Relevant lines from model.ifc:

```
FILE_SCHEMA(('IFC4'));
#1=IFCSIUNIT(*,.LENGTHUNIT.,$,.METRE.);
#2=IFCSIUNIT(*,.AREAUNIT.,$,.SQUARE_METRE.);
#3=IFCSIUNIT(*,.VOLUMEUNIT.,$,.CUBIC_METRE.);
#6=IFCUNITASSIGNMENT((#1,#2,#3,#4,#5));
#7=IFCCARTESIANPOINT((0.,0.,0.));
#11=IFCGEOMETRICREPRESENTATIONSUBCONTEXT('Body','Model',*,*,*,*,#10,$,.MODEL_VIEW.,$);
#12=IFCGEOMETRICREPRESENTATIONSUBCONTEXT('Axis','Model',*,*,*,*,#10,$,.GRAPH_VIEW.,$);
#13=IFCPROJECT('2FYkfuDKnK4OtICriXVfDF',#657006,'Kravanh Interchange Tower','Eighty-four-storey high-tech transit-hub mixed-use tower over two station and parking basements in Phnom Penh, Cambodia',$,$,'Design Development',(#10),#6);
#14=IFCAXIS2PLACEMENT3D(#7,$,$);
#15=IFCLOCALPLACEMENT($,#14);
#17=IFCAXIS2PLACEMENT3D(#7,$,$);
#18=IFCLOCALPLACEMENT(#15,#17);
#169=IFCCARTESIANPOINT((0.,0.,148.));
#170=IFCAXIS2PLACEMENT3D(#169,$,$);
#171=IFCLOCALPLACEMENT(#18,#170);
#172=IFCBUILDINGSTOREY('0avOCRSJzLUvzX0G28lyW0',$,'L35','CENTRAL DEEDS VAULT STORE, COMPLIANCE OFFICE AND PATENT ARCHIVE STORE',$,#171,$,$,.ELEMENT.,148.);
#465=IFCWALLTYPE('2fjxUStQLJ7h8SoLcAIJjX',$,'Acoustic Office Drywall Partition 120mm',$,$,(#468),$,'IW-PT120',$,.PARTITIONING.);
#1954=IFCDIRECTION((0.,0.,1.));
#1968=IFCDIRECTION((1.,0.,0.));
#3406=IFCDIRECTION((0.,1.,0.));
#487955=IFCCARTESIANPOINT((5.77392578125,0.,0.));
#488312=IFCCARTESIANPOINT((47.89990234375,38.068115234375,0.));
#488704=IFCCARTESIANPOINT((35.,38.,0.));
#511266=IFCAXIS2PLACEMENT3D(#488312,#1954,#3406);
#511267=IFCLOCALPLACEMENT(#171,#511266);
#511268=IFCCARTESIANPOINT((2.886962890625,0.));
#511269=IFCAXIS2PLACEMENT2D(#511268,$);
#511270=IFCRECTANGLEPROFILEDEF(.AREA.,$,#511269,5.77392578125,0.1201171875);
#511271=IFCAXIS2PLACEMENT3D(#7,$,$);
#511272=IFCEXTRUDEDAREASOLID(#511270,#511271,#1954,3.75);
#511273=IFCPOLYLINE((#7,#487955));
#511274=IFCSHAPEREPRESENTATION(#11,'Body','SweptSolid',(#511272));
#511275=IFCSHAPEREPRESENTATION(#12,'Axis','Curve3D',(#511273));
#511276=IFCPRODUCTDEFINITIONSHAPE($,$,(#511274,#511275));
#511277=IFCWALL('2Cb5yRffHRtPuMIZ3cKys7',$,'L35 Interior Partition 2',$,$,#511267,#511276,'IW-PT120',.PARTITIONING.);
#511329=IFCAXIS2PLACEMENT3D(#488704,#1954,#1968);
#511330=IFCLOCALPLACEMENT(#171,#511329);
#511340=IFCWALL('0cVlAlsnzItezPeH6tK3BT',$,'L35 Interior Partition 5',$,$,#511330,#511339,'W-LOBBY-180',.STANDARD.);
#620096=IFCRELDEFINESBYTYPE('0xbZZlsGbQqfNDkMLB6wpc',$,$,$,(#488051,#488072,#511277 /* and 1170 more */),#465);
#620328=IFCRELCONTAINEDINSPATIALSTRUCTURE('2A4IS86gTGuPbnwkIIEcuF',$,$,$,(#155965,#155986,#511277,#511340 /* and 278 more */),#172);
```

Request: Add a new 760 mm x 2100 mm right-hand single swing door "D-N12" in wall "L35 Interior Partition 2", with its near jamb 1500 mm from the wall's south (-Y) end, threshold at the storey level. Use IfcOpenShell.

```python
import numpy as np
import ifcopenshell
import ifcopenshell.api.feature
import ifcopenshell.api.geometry
import ifcopenshell.api.root
import ifcopenshell.api.spatial
import ifcopenshell.geom
import ifcopenshell.util.element
import ifcopenshell.util.placement
import ifcopenshell.util.representation
import ifcopenshell.util.shape
import ifcopenshell.util.unit

model = ifcopenshell.open("model.ifc")
unit_scale = ifcopenshell.util.unit.calculate_unit_scale(model)
settings = ifcopenshell.geom.settings()


def volume(element):
    """Net volume in cubic metres, openings subtracted."""
    shape = ifcopenshell.geom.create_shape(settings, element)
    return ifcopenshell.util.shape.get_volume(shape.geometry)


wall = model.by_id(511277)
storey = ifcopenshell.util.element.get_container(wall, ifc_class="IfcBuildingStorey")
context = ifcopenshell.util.representation.get_context(model, "Model", "Body", "MODEL_VIEW")
before = volume(wall)

width, height, from_end, sill = 0.76, 2.1, 1.5, 0.0  # metres

# The wall runs along its own X axis, and the end named is its -X end.
wall_shape = ifcopenshell.geom.create_shape(settings, wall)
x, y, z = ifcopenshell.util.shape.get_vertices(wall_shape.geometry).T
start = x.min() + from_end
face, thickness = float(y.min()), float(y.max() - y.min())
wall_matrix = ifcopenshell.util.placement.get_local_placement(wall.ObjectPlacement)
level = ifcopenshell.util.placement.get_local_placement(storey.ObjectPlacement)[2, 3]


def in_wall(x, y):
    """Placement at x, y metres in the wall's axes, at sill height."""
    matrix = wall_matrix.copy()
    matrix[:, 3] = wall_matrix @ np.array([x / unit_scale, y / unit_scale, 0.0, 1.0])
    matrix[2, 3] = level + sill / unit_scale
    return matrix


# Opening: a box that overshoots both wall faces by 50 mm.
opening = ifcopenshell.api.root.create_entity(model, ifc_class="IfcOpeningElement", predefined_type="OPENING")
box = ifcopenshell.api.geometry.add_wall_representation(
    model, context=context, length=width, height=height, thickness=thickness + 0.1
)
ifcopenshell.api.geometry.assign_representation(model, product=opening, representation=box)
ifcopenshell.api.geometry.edit_object_placement(model, product=opening, matrix=in_wall(start, face - 0.05), is_si=False)
ifcopenshell.api.feature.add_feature(model, feature=opening, element=wall)

door = ifcopenshell.api.root.create_entity(model, ifc_class="IfcDoor", name="D-N12", predefined_type="DOOR")
door.OverallWidth, door.OverallHeight = width / unit_scale, height / unit_scale
door.OperationType = "SINGLE_SWING_RIGHT"
body = ifcopenshell.api.geometry.add_door_representation(
    model,
    context=context,
    overall_width=door.OverallWidth,
    overall_height=door.OverallHeight,
    operation_type="SINGLE_SWING_RIGHT",
    lining_properties={"LiningDepth": thickness / unit_scale, "ThresholdDepth": thickness / unit_scale},
)
ifcopenshell.api.geometry.assign_representation(model, product=door, representation=body)
ifcopenshell.api.spatial.assign_container(model, products=[door], relating_structure=storey)
ifcopenshell.api.feature.add_filling(model, opening=opening, element=door)

# The lining spans the wall, so the door starts at the wall face.
ifcopenshell.api.geometry.edit_object_placement(model, product=door, matrix=in_wall(start, face), is_si=False)

after = volume(wall)

print(f"wall volume {before:.3f} -> {after:.3f} m3")

model.write("model_rev.ifc")
```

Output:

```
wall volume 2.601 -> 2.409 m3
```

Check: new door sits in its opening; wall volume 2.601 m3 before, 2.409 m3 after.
